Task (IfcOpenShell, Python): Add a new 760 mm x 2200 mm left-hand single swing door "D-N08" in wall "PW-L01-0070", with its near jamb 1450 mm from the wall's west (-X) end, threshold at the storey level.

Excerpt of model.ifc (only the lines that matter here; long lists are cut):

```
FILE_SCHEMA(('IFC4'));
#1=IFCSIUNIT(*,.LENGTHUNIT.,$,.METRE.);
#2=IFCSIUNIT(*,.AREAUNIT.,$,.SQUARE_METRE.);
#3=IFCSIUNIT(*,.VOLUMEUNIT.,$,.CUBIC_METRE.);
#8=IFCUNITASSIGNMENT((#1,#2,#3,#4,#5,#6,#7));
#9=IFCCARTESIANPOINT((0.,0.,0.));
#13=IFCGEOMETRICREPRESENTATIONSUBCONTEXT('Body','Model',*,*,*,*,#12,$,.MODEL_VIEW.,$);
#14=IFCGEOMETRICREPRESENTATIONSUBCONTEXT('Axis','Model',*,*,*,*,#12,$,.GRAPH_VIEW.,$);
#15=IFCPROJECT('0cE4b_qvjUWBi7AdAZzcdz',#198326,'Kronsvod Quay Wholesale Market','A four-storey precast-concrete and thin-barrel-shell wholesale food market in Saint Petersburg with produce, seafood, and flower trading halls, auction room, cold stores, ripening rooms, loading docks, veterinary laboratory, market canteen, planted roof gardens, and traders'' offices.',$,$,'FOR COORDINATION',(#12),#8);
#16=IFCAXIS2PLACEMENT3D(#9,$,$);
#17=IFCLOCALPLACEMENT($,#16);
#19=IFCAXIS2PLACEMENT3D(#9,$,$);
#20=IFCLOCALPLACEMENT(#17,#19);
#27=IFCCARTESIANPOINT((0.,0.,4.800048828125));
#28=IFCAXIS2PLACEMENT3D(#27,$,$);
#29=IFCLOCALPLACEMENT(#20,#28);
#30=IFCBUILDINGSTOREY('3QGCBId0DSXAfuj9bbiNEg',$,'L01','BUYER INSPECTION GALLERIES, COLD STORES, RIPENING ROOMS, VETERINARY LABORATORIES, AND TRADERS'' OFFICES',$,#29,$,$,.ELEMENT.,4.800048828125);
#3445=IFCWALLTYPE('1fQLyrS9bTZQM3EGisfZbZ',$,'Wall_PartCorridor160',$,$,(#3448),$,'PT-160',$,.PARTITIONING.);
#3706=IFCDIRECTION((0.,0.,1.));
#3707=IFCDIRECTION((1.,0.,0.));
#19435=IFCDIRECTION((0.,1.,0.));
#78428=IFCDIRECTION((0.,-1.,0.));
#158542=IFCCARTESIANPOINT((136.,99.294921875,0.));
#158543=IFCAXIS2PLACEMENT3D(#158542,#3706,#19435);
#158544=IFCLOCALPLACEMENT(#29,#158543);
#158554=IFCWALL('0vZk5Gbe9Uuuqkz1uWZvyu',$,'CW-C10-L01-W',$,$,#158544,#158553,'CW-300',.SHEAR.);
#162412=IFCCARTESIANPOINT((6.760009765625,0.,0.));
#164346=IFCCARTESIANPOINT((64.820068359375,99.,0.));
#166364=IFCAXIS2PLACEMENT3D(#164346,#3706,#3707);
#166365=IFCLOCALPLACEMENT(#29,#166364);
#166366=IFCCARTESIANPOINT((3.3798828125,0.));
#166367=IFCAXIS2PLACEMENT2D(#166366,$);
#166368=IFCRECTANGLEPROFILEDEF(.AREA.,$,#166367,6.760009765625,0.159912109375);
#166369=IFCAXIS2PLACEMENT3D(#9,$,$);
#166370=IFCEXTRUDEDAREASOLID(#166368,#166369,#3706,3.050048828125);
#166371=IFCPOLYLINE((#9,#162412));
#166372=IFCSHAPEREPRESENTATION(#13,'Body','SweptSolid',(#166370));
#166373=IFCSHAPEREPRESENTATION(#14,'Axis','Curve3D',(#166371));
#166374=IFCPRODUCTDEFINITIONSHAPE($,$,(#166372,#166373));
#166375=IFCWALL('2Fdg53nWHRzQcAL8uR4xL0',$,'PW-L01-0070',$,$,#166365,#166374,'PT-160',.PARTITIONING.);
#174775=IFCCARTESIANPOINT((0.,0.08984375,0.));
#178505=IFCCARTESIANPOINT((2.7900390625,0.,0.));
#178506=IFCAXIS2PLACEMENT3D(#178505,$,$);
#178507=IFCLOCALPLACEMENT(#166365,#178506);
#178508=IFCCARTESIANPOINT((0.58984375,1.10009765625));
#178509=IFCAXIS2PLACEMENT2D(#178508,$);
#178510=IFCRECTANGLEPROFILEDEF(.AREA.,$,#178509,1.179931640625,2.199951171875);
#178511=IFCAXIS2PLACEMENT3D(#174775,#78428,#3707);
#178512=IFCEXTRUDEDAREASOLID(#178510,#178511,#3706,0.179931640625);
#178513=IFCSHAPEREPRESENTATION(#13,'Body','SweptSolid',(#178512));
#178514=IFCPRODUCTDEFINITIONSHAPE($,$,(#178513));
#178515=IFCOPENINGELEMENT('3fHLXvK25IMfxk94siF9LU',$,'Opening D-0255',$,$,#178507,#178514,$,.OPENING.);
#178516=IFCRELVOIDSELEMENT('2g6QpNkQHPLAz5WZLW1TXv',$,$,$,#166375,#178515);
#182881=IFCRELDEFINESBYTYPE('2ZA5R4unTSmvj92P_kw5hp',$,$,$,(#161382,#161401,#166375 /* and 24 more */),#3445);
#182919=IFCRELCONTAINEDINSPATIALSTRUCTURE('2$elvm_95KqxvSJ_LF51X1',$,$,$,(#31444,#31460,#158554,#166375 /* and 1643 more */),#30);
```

```python
import numpy as np
import ifcopenshell
import ifcopenshell.api.feature
import ifcopenshell.api.geometry
import ifcopenshell.api.root
import ifcopenshell.api.spatial
import ifcopenshell.geom
import ifcopenshell.util.element
import ifcopenshell.util.placement
import ifcopenshell.util.representation
import ifcopenshell.util.shape
import ifcopenshell.util.unit

model = ifcopenshell.open("model.ifc")
unit_scale = ifcopenshell.util.unit.calculate_unit_scale(model)
settings = ifcopenshell.geom.settings()


def volume(element):
    """Net volume in cubic metres, openings subtracted."""
    shape = ifcopenshell.geom.create_shape(settings, element)
    return ifcopenshell.util.shape.get_volume(shape.geometry)


wall = model.by_id(166375)
storey = ifcopenshell.util.element.get_container(wall, ifc_class="IfcBuildingStorey")
context = ifcopenshell.util.representation.get_context(model, "Model", "Body", "MODEL_VIEW")
before = volume(wall)

width, height, from_end, sill = 0.76, 2.2, 1.45, 0.0  # metres

# The wall runs along its own X axis, and the end named is its -X end.
wall_shape = ifcopenshell.geom.create_shape(settings, wall)
x, y, z = ifcopenshell.util.shape.get_vertices(wall_shape.geometry).T
start = x.min() + from_end
face, thickness = float(y.min()), float(y.max() - y.min())
wall_matrix = ifcopenshell.util.placement.get_local_placement(wall.ObjectPlacement)
level = ifcopenshell.util.placement.get_local_placement(storey.ObjectPlacement)[2, 3]


def in_wall(x, y):
    """Placement at x, y metres in the wall's axes, at sill height."""
    matrix = wall_matrix.copy()
    matrix[:, 3] = wall_matrix @ np.array([x / unit_scale, y / unit_scale, 0.0, 1.0])
    matrix[2, 3] = level + sill / unit_scale
    return matrix


# Opening: a box that overshoots both wall faces by 50 mm.
opening = ifcopenshell.api.root.create_entity(model, ifc_class="IfcOpeningElement", predefined_type="OPENING")
box = ifcopenshell.api.geometry.add_wall_representation(
    model, context=context, length=width, height=height, thickness=thickness + 0.1
)
ifcopenshell.api.geometry.assign_representation(model, product=opening, representation=box)
ifcopenshell.api.geometry.edit_object_placement(model, product=opening, matrix=in_wall(start, face - 0.05), is_si=False)
ifcopenshell.api.feature.add_feature(model, feature=opening, element=wall)

door = ifcopenshell.api.root.create_entity(model, ifc_class="IfcDoor", name="D-N08", predefined_type="DOOR")
door.OverallWidth, door.OverallHeight = width / unit_scale, height / unit_scale
door.OperationType = "SINGLE_SWING_LEFT"
body = ifcopenshell.api.geometry.add_door_representation(
    model,
    context=context,
    overall_width=door.OverallWidth,
    overall_height=door.OverallHeight,
    operation_type="SINGLE_SWING_LEFT",
    lining_properties={"LiningDepth": thickness / unit_scale, "ThresholdDepth": thickness / unit_scale},
)
ifcopenshell.api.geometry.assign_representation(model, product=door, representation=body)
ifcopenshell.api.spatial.assign_container(model, products=[door], relating_structure=storey)
ifcopenshell.api.feature.add_filling(model, opening=opening, element=door)

# The lining spans the wall, so the door starts at the wall face.
ifcopenshell.api.geometry.edit_object_placement(model, product=door, matrix=in_wall(start, face), is_si=False)

after = volume(wall)

print(f"wall volume {before:.3f} -> {after:.3f} m3")

model.write("model_edited.ifc")
```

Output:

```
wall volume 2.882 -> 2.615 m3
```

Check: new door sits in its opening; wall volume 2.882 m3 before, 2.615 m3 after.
